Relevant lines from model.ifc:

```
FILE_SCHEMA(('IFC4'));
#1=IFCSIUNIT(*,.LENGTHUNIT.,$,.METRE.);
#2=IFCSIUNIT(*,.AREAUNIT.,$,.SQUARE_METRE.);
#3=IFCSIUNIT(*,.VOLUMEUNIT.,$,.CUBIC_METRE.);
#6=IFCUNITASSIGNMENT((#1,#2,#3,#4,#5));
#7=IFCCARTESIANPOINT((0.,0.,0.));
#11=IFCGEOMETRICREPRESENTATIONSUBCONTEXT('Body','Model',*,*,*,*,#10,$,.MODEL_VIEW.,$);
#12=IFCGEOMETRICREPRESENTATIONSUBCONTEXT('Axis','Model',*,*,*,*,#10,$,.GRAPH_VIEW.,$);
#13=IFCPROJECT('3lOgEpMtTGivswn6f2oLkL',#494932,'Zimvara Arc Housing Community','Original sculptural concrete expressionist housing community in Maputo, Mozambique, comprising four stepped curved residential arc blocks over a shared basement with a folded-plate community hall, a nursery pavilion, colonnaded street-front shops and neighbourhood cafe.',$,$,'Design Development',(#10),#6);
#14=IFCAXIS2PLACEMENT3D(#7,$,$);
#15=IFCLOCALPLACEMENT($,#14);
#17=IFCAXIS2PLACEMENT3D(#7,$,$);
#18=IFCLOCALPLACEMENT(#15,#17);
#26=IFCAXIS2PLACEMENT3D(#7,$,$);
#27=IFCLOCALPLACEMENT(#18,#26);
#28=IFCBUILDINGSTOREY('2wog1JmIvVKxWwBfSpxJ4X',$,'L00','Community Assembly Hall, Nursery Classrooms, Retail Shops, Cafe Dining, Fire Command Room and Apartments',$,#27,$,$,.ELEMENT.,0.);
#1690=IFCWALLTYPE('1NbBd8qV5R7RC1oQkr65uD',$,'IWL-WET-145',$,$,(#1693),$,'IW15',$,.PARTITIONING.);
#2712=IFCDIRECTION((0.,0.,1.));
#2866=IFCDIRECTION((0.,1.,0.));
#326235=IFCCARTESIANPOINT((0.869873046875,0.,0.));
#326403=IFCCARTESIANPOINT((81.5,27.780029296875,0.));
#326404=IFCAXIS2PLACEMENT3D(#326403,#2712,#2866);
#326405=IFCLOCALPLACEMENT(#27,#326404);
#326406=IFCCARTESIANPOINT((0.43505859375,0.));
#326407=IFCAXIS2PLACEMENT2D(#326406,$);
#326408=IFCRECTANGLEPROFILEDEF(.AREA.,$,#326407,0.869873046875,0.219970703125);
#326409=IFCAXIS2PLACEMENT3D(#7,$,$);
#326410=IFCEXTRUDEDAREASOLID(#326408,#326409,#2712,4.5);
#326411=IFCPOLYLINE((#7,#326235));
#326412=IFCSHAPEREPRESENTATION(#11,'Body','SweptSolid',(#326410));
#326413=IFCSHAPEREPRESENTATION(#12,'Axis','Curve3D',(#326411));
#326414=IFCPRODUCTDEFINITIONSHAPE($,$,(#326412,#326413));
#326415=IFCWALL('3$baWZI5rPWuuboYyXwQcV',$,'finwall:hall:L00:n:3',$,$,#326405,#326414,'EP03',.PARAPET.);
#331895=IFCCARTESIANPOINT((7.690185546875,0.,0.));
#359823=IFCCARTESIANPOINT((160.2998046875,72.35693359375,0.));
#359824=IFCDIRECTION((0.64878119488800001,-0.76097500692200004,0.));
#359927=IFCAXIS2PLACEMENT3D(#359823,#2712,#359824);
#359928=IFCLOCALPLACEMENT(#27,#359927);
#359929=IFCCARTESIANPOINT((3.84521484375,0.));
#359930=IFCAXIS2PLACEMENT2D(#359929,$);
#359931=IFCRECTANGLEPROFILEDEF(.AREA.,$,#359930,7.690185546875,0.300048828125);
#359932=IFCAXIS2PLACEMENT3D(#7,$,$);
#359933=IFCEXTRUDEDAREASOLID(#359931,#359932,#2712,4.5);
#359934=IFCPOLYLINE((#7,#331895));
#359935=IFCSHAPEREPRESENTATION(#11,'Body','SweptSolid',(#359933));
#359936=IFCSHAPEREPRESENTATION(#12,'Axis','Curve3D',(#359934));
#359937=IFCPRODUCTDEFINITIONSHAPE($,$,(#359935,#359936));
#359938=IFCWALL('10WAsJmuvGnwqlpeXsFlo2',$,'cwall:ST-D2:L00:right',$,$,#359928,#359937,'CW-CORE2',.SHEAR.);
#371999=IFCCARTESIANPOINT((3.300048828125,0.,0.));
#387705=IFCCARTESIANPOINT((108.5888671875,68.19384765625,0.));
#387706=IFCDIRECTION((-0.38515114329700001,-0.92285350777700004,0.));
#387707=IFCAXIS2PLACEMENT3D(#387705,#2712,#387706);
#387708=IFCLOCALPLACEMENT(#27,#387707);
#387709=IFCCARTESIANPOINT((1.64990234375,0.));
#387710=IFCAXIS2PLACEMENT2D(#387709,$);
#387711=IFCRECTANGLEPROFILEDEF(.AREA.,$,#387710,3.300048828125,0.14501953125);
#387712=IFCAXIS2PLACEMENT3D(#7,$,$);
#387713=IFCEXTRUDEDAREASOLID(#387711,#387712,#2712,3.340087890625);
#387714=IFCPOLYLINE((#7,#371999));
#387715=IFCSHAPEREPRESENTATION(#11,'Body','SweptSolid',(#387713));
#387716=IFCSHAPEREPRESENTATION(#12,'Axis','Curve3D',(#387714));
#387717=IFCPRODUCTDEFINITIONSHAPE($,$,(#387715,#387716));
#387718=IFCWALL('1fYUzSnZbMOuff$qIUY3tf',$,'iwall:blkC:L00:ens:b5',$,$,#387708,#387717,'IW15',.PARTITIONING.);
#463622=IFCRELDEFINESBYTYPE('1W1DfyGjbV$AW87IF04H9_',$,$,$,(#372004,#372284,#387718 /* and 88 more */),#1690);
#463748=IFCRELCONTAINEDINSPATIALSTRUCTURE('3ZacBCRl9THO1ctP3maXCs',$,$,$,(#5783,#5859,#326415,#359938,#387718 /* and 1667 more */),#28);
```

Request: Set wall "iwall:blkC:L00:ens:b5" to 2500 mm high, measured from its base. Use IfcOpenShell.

```python
import ifcopenshell
import ifcopenshell.geom
import ifcopenshell.util.representation
import ifcopenshell.util.shape

model = ifcopenshell.open("model.ifc")
settings = ifcopenshell.geom.settings()


def volume(element):
    """Net volume in cubic metres, openings subtracted."""
    shape = ifcopenshell.geom.create_shape(settings, element)
    return ifcopenshell.util.shape.get_volume(shape.geometry)


wall = model.by_id(387718)
before = volume(wall)

body = ifcopenshell.util.representation.get_representation(wall, "Model", "Body")
solid = body.Items[0]
old_height = solid.Depth
solid.Depth = 2.5
after = volume(wall)

print(f"height {old_height:g} -> {solid.Depth:g}, volume {before:.3f} -> {after:.3f} m3")

model.write("model_updated.ifc")
```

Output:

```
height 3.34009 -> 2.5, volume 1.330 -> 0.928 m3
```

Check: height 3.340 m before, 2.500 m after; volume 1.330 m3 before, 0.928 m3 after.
